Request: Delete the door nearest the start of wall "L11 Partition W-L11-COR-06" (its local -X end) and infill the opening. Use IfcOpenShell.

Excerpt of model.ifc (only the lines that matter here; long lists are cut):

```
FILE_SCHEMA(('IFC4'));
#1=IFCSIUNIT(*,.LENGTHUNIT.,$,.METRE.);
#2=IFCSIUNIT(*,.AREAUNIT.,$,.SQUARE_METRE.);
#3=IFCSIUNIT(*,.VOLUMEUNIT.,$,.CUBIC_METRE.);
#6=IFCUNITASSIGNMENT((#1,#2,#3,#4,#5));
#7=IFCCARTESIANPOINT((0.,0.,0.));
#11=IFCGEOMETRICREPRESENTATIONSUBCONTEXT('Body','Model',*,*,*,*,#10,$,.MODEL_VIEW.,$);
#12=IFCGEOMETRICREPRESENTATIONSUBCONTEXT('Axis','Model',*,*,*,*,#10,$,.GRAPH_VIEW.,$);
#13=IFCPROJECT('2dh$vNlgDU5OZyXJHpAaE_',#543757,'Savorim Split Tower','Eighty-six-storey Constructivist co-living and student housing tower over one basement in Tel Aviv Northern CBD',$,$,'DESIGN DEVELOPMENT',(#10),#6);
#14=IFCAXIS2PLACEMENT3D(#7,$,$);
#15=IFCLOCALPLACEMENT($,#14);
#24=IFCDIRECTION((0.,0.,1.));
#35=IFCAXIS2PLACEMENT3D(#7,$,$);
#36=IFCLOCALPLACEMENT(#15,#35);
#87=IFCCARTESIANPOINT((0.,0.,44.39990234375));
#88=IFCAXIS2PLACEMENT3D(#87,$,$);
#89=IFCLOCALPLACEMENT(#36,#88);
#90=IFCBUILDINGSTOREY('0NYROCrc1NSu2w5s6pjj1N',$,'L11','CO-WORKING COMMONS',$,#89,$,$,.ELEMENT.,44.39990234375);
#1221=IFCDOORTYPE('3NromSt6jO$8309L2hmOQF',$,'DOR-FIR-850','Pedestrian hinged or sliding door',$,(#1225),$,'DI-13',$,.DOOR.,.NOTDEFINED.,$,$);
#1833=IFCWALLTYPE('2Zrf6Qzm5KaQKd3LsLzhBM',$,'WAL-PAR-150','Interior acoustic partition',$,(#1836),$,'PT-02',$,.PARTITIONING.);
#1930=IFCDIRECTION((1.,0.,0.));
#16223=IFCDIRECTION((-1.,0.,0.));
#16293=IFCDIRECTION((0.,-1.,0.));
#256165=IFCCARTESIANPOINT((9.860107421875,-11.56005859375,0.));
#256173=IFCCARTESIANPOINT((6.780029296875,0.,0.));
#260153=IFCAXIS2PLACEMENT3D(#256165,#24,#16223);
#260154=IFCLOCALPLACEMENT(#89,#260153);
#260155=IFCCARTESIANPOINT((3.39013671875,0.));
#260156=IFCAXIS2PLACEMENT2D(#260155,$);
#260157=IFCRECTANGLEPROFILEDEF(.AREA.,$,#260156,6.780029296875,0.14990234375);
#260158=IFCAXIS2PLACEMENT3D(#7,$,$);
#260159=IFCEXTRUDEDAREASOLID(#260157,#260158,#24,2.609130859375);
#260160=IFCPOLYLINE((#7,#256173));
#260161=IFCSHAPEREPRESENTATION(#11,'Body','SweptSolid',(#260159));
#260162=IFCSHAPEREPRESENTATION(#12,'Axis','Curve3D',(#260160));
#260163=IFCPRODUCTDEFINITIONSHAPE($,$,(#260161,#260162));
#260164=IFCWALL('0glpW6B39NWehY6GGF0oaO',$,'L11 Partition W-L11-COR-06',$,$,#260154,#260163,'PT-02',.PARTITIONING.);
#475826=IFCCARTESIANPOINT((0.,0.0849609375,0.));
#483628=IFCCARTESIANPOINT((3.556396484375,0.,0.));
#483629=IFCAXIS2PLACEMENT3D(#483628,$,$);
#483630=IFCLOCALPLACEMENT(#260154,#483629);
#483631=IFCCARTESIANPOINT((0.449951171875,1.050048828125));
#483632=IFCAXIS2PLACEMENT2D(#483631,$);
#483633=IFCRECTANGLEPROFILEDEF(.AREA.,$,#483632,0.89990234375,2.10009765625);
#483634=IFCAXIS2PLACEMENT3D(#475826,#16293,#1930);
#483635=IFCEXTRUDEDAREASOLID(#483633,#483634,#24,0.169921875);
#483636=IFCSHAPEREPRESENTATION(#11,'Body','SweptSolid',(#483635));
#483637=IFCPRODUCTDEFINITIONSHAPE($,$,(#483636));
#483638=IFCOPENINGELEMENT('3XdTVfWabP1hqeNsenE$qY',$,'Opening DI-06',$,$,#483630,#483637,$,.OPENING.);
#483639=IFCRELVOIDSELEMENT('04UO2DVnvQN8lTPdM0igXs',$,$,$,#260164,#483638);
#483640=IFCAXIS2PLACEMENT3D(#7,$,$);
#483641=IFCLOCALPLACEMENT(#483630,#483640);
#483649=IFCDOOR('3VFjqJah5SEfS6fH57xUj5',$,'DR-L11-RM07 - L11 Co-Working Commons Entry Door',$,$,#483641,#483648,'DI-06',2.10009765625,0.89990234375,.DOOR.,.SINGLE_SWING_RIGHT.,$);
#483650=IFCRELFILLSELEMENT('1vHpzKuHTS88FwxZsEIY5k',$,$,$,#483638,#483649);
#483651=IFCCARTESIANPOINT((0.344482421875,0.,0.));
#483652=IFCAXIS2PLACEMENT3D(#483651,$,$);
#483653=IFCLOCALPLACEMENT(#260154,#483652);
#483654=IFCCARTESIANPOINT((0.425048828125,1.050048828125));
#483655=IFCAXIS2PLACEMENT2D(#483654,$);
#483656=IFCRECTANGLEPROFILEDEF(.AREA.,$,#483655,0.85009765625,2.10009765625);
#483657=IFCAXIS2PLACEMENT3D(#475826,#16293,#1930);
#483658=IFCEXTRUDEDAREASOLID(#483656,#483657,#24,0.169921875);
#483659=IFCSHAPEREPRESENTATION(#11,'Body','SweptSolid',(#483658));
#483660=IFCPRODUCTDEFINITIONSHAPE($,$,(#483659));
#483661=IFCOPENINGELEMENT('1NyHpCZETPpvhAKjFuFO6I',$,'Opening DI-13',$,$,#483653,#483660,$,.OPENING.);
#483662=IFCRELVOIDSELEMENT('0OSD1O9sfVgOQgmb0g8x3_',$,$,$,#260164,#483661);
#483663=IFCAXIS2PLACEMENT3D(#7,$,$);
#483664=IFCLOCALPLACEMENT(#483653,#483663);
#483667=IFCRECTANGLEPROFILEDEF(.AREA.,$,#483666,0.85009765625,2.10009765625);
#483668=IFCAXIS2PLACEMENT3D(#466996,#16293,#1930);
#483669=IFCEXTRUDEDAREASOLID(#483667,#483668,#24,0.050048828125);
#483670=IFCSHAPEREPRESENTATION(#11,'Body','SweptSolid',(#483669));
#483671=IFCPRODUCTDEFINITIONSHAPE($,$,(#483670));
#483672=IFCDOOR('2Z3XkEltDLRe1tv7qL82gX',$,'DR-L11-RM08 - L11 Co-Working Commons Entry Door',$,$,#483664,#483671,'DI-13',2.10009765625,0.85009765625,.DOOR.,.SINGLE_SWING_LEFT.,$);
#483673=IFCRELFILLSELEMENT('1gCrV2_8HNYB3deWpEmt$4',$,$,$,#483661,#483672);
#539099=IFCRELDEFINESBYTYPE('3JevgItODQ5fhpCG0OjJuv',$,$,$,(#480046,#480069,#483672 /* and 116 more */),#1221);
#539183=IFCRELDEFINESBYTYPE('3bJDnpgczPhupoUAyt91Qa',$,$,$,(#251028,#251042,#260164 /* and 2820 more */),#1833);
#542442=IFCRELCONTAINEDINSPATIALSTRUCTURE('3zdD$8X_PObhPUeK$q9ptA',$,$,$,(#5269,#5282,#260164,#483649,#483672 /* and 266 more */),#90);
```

```python
import ifcopenshell
import ifcopenshell.api.feature
import ifcopenshell.api.root
import ifcopenshell.geom
import ifcopenshell.util.shape

model = ifcopenshell.open("model.ifc")
settings = ifcopenshell.geom.settings()


def volume(element):
    """Net volume in cubic metres, openings subtracted."""
    shape = ifcopenshell.geom.create_shape(settings, element)
    return ifcopenshell.util.shape.get_volume(shape.geometry)


door = model.by_id(483672)
opening = door.FillsVoids[0].RelatingOpeningElement
wall = opening.VoidsElements[0].RelatingBuildingElement
before = volume(wall)

ifcopenshell.api.root.remove_product(model, product=door)
ifcopenshell.api.feature.remove_feature(model, feature=opening)

after = volume(wall)

print(f"wall volume {before:.3f} -> {after:.3f} m3")

model.write("model-out.ifc")
```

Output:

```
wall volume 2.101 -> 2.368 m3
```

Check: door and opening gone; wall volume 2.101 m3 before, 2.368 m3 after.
